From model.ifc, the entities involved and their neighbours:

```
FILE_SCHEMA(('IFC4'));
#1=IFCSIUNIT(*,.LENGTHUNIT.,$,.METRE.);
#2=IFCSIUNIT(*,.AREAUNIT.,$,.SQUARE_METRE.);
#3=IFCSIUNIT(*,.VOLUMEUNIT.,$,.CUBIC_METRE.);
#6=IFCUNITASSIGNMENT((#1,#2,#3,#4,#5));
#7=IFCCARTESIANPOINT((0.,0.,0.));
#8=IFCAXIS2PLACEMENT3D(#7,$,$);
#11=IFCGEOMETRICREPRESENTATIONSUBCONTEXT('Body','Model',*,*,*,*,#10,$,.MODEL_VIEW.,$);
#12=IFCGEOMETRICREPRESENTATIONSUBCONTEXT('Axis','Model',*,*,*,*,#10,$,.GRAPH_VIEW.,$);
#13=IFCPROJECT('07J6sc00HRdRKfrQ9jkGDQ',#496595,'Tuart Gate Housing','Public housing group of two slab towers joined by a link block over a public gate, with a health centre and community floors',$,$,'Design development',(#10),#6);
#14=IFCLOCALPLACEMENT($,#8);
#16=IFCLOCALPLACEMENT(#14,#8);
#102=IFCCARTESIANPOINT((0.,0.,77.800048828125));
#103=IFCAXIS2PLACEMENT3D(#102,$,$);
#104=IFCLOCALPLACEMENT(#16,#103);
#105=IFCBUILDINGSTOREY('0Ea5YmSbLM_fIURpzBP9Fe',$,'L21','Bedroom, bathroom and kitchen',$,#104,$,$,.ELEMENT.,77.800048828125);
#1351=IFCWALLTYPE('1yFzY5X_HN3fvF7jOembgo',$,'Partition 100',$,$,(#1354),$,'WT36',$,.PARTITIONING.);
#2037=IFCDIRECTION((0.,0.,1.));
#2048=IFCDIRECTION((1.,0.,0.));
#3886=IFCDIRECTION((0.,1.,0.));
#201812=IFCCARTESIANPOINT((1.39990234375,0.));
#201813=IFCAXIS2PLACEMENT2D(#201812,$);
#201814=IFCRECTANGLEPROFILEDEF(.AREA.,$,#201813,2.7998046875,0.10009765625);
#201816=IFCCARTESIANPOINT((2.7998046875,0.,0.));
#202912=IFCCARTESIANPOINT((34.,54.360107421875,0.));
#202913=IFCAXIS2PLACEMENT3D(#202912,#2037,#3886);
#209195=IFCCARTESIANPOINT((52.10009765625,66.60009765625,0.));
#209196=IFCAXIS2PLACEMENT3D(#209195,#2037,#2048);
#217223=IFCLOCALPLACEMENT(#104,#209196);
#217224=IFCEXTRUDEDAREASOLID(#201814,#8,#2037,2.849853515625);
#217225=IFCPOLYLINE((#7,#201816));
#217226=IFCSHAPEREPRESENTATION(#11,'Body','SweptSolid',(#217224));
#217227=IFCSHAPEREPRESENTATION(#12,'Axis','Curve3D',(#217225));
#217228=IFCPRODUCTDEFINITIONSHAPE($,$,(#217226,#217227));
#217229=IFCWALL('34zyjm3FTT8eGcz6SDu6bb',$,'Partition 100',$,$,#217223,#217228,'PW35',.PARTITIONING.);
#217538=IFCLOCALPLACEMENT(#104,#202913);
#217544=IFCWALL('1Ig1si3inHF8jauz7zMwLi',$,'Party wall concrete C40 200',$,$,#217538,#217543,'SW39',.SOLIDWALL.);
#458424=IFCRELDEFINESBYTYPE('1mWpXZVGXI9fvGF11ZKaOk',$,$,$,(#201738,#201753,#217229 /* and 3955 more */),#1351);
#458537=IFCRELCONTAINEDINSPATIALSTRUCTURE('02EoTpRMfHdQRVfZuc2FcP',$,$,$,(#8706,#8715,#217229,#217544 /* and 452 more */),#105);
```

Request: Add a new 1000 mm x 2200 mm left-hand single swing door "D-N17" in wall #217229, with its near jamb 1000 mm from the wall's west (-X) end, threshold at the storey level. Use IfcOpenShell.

```python
import numpy as np
import ifcopenshell
import ifcopenshell.api.feature
import ifcopenshell.api.geometry
import ifcopenshell.api.root
import ifcopenshell.api.spatial
import ifcopenshell.geom
import ifcopenshell.util.element
import ifcopenshell.util.placement
import ifcopenshell.util.representation
import ifcopenshell.util.shape
import ifcopenshell.util.unit

model = ifcopenshell.open("model.ifc")
unit_scale = ifcopenshell.util.unit.calculate_unit_scale(model)
settings = ifcopenshell.geom.settings()


def volume(element):
    """Net volume in cubic metres, openings subtracted."""
    shape = ifcopenshell.geom.create_shape(settings, element)
    return ifcopenshell.util.shape.get_volume(shape.geometry)


wall = model.by_guid("34zyjm3FTT8eGcz6SDu6bb")
storey = ifcopenshell.util.element.get_container(wall, ifc_class="IfcBuildingStorey")
context = ifcopenshell.util.representation.get_context(model, "Model", "Body", "MODEL_VIEW")
before = volume(wall)

width, height, from_end, sill = 1, 2.2, 1, 0.0  # metres

# The wall runs along its own X axis, and the end named is its -X end.
wall_shape = ifcopenshell.geom.create_shape(settings, wall)
x, y, z = ifcopenshell.util.shape.get_vertices(wall_shape.geometry).T
start = x.min() + from_end
face, thickness = float(y.min()), float(y.max() - y.min())
wall_matrix = ifcopenshell.util.placement.get_local_placement(wall.ObjectPlacement)
level = ifcopenshell.util.placement.get_local_placement(storey.ObjectPlacement)[2, 3]


def in_wall(x, y):
    """Placement at x, y metres in the wall's axes, at sill height."""
    matrix = wall_matrix.copy()
    matrix[:, 3] = wall_matrix @ np.array([x / unit_scale, y / unit_scale, 0.0, 1.0])
    matrix[2, 3] = level + sill / unit_scale
    return matrix


# Opening: a box that overshoots both wall faces by 50 mm.
opening = ifcopenshell.api.root.create_entity(model, ifc_class="IfcOpeningElement", predefined_type="OPENING")
box = ifcopenshell.api.geometry.add_wall_representation(
    model, context=context, length=width, height=height, thickness=thickness + 0.1
)
ifcopenshell.api.geometry.assign_representation(model, product=opening, representation=box)
ifcopenshell.api.geometry.edit_object_placement(model, product=opening, matrix=in_wall(start, face - 0.05), is_si=False)
ifcopenshell.api.feature.add_feature(model, feature=opening, element=wall)

door = ifcopenshell.api.root.create_entity(model, ifc_class="IfcDoor", name="D-N17", predefined_type="DOOR")
door.OverallWidth, door.OverallHeight = width / unit_scale, height / unit_scale
door.OperationType = "SINGLE_SWING_LEFT"
body = ifcopenshell.api.geometry.add_door_representation(
    model,
    context=context,
    overall_width=door.OverallWidth,
    overall_height=door.OverallHeight,
    operation_type="SINGLE_SWING_LEFT",
    lining_properties={"LiningDepth": thickness / unit_scale, "ThresholdDepth": thickness / unit_scale},
)
ifcopenshell.api.geometry.assign_representation(model, product=door, representation=body)
ifcopenshell.api.spatial.assign_container(model, products=[door], relating_structure=storey)
ifcopenshell.api.feature.add_filling(model, opening=opening, element=door)

# The lining spans the wall, so the door starts at the wall face.
ifcopenshell.api.geometry.edit_object_placement(model, product=door, matrix=in_wall(start, face), is_si=False)

after = volume(wall)

print(f"wall volume {before:.3f} -> {after:.3f} m3")

model.write("model-out.ifc")
```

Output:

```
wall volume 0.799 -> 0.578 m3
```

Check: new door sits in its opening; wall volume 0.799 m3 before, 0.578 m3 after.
